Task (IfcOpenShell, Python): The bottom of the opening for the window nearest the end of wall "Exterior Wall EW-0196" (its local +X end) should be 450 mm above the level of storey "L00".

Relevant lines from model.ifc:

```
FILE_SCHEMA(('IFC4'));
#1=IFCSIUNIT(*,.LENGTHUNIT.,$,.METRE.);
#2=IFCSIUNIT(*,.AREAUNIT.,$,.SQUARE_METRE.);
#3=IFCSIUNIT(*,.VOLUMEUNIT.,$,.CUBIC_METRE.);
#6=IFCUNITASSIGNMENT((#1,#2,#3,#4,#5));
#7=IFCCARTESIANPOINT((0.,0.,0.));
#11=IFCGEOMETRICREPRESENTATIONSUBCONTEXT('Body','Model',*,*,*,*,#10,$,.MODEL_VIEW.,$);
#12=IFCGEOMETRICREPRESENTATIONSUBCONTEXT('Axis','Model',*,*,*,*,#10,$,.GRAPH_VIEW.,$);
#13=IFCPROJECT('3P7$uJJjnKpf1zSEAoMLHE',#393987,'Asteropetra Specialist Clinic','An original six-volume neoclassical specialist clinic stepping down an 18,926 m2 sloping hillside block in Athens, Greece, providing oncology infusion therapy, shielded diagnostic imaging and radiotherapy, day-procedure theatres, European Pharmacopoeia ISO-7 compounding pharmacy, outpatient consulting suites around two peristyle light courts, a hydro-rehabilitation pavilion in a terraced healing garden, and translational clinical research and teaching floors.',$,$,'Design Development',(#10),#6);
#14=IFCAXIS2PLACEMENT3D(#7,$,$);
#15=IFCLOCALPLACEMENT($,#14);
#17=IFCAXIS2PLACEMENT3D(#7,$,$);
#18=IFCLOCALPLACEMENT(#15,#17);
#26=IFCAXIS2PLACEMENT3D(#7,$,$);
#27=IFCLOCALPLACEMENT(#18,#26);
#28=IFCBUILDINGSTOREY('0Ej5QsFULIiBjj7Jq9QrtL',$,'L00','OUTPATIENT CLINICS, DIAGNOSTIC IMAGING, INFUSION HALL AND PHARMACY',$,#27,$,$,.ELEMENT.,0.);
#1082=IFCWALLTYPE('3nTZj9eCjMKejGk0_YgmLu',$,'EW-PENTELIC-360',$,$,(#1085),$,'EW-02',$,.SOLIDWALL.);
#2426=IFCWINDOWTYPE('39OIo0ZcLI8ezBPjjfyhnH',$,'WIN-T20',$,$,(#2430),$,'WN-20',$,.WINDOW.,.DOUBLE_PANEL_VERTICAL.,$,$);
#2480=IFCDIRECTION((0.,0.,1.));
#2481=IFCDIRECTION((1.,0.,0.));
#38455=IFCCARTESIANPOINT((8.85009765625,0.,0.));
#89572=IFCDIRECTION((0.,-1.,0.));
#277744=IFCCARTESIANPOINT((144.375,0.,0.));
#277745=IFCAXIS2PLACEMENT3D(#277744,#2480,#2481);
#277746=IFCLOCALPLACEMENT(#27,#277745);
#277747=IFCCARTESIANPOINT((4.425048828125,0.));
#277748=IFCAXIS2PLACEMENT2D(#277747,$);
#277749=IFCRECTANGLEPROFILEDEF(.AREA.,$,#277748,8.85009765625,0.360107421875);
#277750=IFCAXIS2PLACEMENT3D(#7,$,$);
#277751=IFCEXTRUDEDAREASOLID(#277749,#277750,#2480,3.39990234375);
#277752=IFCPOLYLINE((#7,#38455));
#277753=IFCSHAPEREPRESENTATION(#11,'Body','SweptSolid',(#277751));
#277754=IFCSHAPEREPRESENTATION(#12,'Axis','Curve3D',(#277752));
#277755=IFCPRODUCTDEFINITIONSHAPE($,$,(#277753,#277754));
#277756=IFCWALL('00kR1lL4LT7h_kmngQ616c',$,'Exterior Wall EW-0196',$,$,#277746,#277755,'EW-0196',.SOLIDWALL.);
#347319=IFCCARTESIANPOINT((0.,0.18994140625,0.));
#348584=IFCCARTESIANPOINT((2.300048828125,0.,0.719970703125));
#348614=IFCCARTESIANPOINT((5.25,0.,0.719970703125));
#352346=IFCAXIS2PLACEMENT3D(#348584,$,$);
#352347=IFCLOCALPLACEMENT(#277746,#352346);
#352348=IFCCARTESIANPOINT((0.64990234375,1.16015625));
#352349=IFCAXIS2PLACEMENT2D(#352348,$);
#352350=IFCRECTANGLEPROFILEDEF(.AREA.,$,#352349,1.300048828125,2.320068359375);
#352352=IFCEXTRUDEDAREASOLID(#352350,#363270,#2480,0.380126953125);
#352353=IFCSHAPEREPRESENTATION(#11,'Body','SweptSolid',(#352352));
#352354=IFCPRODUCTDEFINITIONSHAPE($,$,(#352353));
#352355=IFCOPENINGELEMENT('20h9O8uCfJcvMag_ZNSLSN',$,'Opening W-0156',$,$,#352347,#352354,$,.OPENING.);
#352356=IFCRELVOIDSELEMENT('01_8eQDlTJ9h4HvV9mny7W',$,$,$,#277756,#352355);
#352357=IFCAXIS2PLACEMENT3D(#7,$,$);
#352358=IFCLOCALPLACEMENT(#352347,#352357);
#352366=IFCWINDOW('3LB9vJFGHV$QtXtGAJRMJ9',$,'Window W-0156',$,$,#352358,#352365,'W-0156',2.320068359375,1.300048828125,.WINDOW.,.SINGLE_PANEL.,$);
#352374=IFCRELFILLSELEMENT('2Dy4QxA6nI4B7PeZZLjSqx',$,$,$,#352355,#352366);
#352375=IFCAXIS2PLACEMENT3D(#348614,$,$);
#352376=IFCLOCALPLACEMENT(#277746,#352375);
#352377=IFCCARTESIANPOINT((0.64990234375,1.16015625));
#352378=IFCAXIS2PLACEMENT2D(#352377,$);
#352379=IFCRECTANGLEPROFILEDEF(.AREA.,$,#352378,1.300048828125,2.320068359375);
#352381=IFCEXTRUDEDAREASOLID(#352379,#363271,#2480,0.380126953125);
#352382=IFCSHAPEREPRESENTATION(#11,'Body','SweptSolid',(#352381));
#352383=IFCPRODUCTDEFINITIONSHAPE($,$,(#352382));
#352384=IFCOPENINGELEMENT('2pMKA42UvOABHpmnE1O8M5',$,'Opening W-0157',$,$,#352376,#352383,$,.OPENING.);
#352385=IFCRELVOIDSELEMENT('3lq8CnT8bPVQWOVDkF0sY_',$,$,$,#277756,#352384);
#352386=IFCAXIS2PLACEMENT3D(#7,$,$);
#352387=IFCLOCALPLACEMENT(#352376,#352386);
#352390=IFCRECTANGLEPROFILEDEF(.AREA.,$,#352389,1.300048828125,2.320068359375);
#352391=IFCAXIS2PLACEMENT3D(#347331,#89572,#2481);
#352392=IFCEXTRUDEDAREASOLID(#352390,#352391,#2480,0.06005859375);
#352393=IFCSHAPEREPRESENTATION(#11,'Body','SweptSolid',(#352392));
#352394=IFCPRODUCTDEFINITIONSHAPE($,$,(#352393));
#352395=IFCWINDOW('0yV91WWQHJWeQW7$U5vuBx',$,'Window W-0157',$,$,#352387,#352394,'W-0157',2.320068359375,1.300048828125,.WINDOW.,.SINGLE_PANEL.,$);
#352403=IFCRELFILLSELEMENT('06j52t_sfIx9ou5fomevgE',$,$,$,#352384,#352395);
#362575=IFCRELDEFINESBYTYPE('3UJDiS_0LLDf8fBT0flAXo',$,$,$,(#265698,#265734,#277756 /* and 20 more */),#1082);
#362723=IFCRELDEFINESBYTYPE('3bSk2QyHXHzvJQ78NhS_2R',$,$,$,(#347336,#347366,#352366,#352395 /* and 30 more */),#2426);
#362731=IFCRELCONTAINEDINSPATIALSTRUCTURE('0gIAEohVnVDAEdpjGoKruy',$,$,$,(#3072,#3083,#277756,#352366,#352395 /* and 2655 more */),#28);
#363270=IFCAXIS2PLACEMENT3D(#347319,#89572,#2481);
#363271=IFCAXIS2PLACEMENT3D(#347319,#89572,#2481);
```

```python
import numpy as np
import ifcopenshell
import ifcopenshell.api.geometry
import ifcopenshell.geom
import ifcopenshell.util.element
import ifcopenshell.util.placement
import ifcopenshell.util.shape
import ifcopenshell.util.unit

model = ifcopenshell.open("model.ifc")
unit_scale = ifcopenshell.util.unit.calculate_unit_scale(model)

window = model.by_guid("0yV91WWQHJWeQW7$U5vuBx")
opening = window.FillsVoids[0].RelatingOpeningElement
storey = ifcopenshell.util.element.get_container(window, ifc_class="IfcBuildingStorey")
level = ifcopenshell.util.placement.get_local_placement(storey.ObjectPlacement)[2, 3]

# The opening's origin need not be at the sill, so measure its lowest point.
shape = ifcopenshell.geom.create_shape(ifcopenshell.geom.settings(), opening)
bottom = ifcopenshell.util.shape.get_shape_bottom_elevation(shape, shape.geometry) / unit_scale
dz = level + 0.45 / unit_scale - bottom

shift = np.array([0.0, 0.0, dz])
# The window is placed relative to its opening, so it follows when the opening moves.
matrix = ifcopenshell.util.placement.get_local_placement(opening.ObjectPlacement)
matrix[:3, 3] += shift
ifcopenshell.api.geometry.edit_object_placement(
    model, product=opening, matrix=matrix, is_si=False, should_transform_children=True
)

print(f"moved by {dz * unit_scale:+.3f} m")

model.write("model_updated.ifc")
```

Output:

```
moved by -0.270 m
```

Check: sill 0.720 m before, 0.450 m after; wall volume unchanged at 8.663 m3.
